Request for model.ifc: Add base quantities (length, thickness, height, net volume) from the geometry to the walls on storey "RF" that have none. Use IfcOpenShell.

First a look at what the model holds.

```python
import ifcopenshell
import ifcopenshell.util.element
import ifcopenshell.util.unit

model = ifcopenshell.open("model.ifc")
print(model.schema)
for unit_type in ("LENGTHUNIT", "AREAUNIT", "VOLUMEUNIT"):
    print(unit_type, ifcopenshell.util.unit.calculate_unit_scale(model, unit_type))
storey = next(s for s in model.by_type("IfcBuildingStorey") if s.Name == "RF")
walls = [e for e in ifcopenshell.util.element.get_decomposition(storey) if e.is_a("IfcWall")]
for e in sorted(walls, key=lambda e: e.id()):
    print(e.id(), e.is_a(), e.Name, list(ifcopenshell.util.element.get_psets(e, qtos_only=True)), sep=" | ")
```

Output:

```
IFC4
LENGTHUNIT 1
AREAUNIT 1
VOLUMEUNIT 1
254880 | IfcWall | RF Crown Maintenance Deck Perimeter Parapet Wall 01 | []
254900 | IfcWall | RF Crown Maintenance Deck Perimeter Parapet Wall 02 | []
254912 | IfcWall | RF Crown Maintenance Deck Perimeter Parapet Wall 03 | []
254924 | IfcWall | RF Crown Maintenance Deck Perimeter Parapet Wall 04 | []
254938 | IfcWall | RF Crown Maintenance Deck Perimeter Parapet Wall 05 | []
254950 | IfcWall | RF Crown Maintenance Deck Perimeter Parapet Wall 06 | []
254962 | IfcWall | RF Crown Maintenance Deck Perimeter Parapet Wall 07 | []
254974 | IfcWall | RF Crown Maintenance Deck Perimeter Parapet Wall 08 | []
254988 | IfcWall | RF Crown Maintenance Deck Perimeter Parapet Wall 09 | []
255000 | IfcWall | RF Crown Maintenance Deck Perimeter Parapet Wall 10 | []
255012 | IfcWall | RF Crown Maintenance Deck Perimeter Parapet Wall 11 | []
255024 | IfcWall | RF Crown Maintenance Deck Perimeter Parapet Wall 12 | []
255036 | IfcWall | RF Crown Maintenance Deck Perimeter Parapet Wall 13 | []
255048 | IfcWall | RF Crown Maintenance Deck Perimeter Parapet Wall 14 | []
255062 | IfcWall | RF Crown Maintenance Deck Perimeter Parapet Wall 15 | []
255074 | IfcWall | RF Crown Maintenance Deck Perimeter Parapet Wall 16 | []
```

```python
import ifcopenshell
import ifcopenshell.api.pset
import ifcopenshell.geom
import ifcopenshell.util.element
import ifcopenshell.util.shape
import ifcopenshell.util.unit

model = ifcopenshell.open("model.ifc")
unit_scale = ifcopenshell.util.unit.calculate_unit_scale(model)
volume_scale = ifcopenshell.util.unit.calculate_unit_scale(model, "VOLUMEUNIT")
settings = ifcopenshell.geom.settings()

storey = next(s for s in model.by_type("IfcBuildingStorey") if s.Name == "RF")
walls = [e for e in ifcopenshell.util.element.get_decomposition(storey) if e.is_a("IfcWall")]

for e in sorted(walls, key=lambda e: e.id()):
    if ifcopenshell.util.element.get_psets(e, qtos_only=True, should_inherit=False):
        continue
    # Geometry comes back in metres, in the element's own axes.
    shape = ifcopenshell.geom.create_shape(settings, e)
    values = {
        "Length": ifcopenshell.util.shape.get_x(shape.geometry) / unit_scale,
        "Width": ifcopenshell.util.shape.get_y(shape.geometry) / unit_scale,
        "Height": ifcopenshell.util.shape.get_z(shape.geometry) / unit_scale,
        "NetVolume": ifcopenshell.util.shape.get_volume(shape.geometry) / volume_scale,
    }
    qto = ifcopenshell.api.pset.add_qto(model, product=e, name="Qto_WallBaseQuantities")
    ifcopenshell.api.pset.edit_qto(model, qto=qto, properties=values)
    print(e.id(), {k: round(v, 3) for k, v in values.items()})

model.write("model-out.ifc")
```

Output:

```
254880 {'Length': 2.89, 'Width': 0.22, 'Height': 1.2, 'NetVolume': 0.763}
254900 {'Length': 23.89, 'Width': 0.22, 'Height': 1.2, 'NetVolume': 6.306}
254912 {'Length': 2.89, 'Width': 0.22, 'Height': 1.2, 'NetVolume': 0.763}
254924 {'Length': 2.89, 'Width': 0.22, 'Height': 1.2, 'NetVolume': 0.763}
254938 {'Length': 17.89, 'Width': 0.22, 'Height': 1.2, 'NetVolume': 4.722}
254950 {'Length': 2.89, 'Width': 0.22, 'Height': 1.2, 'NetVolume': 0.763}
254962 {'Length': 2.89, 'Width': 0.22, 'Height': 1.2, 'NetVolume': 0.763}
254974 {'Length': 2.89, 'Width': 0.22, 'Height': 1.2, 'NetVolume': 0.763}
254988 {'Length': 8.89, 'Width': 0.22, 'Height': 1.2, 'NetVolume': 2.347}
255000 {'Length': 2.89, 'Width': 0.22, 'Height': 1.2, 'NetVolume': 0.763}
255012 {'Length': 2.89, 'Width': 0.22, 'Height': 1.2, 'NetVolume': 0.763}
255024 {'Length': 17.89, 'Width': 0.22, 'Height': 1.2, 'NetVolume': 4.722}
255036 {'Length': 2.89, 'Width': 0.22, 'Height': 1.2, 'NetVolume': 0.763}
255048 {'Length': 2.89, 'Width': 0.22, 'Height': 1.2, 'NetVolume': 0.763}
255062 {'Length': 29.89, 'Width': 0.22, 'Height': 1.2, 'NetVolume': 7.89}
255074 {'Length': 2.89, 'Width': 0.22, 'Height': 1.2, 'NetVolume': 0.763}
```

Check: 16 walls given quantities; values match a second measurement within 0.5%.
